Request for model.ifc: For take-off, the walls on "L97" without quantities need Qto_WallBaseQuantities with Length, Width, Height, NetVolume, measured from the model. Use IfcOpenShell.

First a look at what the model holds.

```python
import ifcopenshell
import ifcopenshell.util.element
import ifcopenshell.util.unit

model = ifcopenshell.open("model.ifc")
print(model.schema)
for unit_type in ("LENGTHUNIT", "AREAUNIT", "VOLUMEUNIT"):
    print(unit_type, ifcopenshell.util.unit.calculate_unit_scale(model, unit_type))
storey = next(s for s in model.by_type("IfcBuildingStorey") if s.Name == "L97")
walls = [e for e in ifcopenshell.util.element.get_decomposition(storey) if e.is_a("IfcWall")]
for e in sorted(walls, key=lambda e: e.id()):
    print(e.id(), e.is_a(), e.Name, list(ifcopenshell.util.element.get_psets(e, qtos_only=True)), sep=" | ")
```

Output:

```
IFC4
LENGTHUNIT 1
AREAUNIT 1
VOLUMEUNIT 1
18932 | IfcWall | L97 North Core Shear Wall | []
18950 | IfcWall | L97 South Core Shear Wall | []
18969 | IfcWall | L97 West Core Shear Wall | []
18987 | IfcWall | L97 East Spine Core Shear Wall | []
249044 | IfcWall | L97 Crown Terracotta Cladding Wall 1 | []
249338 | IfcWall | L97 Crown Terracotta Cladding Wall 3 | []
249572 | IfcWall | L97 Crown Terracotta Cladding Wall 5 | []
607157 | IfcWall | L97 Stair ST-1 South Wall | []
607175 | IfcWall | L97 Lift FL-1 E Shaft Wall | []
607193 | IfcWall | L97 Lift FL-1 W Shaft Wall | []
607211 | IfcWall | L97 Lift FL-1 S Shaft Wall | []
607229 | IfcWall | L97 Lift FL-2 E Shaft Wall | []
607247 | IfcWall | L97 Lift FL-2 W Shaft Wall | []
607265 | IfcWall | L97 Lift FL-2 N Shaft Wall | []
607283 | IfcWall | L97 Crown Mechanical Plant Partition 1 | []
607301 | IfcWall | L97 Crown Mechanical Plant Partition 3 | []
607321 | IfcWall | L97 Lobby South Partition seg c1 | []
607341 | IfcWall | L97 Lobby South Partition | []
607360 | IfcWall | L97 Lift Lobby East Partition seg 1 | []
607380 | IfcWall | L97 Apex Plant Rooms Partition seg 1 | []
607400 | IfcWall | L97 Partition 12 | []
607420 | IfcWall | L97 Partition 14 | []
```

```python
import ifcopenshell
import ifcopenshell.api.pset
import ifcopenshell.geom
import ifcopenshell.util.element
import ifcopenshell.util.shape
import ifcopenshell.util.unit

model = ifcopenshell.open("model.ifc")
unit_scale = ifcopenshell.util.unit.calculate_unit_scale(model)
volume_scale = ifcopenshell.util.unit.calculate_unit_scale(model, "VOLUMEUNIT")
settings = ifcopenshell.geom.settings()

storey = next(s for s in model.by_type("IfcBuildingStorey") if s.Name == "L97")
walls = [e for e in ifcopenshell.util.element.get_decomposition(storey) if e.is_a("IfcWall")]

for e in sorted(walls, key=lambda e: e.id()):
    if ifcopenshell.util.element.get_psets(e, qtos_only=True, should_inherit=False):
        continue
    # Geometry comes back in metres, in the element's own axes.
    shape = ifcopenshell.geom.create_shape(settings, e)
    values = {
        "Length": ifcopenshell.util.shape.get_x(shape.geometry) / unit_scale,
        "Width": ifcopenshell.util.shape.get_y(shape.geometry) / unit_scale,
        "Height": ifcopenshell.util.shape.get_z(shape.geometry) / unit_scale,
        "NetVolume": ifcopenshell.util.shape.get_volume(shape.geometry) / volume_scale,
    }
    qto = ifcopenshell.api.pset.add_qto(model, product=e, name="Qto_WallBaseQuantities")
    ifcopenshell.api.pset.edit_qto(model, qto=qto, properties=values)
    print(e.id(), {k: round(v, 3) for k, v in values.items()})

model.write("model_updated.ifc")
```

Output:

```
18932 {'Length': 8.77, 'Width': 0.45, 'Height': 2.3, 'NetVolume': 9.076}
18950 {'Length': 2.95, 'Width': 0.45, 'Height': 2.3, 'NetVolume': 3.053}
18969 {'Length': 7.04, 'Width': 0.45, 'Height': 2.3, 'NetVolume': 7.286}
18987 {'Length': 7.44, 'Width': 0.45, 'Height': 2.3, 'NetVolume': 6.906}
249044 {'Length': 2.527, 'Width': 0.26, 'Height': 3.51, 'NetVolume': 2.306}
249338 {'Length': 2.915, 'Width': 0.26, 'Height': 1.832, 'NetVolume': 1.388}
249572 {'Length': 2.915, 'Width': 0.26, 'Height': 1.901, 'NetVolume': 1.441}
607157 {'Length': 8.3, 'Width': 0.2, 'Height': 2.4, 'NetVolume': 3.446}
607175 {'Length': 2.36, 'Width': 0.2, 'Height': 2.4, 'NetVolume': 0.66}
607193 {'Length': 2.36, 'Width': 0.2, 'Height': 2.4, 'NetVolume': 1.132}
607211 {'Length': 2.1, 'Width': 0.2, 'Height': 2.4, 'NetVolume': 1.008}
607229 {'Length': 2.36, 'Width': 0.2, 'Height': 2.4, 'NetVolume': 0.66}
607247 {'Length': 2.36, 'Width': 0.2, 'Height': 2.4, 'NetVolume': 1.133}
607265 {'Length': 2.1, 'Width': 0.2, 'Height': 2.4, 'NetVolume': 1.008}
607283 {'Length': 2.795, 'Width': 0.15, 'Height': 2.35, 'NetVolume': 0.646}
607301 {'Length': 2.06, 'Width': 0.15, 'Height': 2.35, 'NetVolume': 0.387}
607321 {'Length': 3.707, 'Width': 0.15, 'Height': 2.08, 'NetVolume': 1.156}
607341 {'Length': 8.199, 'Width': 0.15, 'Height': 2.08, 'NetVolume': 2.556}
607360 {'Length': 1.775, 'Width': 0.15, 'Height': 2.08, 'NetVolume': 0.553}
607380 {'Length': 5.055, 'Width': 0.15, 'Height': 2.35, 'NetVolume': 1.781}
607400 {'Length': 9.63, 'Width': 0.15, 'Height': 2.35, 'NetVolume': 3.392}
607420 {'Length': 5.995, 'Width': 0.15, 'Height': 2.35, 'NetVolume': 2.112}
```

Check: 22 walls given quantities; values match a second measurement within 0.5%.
